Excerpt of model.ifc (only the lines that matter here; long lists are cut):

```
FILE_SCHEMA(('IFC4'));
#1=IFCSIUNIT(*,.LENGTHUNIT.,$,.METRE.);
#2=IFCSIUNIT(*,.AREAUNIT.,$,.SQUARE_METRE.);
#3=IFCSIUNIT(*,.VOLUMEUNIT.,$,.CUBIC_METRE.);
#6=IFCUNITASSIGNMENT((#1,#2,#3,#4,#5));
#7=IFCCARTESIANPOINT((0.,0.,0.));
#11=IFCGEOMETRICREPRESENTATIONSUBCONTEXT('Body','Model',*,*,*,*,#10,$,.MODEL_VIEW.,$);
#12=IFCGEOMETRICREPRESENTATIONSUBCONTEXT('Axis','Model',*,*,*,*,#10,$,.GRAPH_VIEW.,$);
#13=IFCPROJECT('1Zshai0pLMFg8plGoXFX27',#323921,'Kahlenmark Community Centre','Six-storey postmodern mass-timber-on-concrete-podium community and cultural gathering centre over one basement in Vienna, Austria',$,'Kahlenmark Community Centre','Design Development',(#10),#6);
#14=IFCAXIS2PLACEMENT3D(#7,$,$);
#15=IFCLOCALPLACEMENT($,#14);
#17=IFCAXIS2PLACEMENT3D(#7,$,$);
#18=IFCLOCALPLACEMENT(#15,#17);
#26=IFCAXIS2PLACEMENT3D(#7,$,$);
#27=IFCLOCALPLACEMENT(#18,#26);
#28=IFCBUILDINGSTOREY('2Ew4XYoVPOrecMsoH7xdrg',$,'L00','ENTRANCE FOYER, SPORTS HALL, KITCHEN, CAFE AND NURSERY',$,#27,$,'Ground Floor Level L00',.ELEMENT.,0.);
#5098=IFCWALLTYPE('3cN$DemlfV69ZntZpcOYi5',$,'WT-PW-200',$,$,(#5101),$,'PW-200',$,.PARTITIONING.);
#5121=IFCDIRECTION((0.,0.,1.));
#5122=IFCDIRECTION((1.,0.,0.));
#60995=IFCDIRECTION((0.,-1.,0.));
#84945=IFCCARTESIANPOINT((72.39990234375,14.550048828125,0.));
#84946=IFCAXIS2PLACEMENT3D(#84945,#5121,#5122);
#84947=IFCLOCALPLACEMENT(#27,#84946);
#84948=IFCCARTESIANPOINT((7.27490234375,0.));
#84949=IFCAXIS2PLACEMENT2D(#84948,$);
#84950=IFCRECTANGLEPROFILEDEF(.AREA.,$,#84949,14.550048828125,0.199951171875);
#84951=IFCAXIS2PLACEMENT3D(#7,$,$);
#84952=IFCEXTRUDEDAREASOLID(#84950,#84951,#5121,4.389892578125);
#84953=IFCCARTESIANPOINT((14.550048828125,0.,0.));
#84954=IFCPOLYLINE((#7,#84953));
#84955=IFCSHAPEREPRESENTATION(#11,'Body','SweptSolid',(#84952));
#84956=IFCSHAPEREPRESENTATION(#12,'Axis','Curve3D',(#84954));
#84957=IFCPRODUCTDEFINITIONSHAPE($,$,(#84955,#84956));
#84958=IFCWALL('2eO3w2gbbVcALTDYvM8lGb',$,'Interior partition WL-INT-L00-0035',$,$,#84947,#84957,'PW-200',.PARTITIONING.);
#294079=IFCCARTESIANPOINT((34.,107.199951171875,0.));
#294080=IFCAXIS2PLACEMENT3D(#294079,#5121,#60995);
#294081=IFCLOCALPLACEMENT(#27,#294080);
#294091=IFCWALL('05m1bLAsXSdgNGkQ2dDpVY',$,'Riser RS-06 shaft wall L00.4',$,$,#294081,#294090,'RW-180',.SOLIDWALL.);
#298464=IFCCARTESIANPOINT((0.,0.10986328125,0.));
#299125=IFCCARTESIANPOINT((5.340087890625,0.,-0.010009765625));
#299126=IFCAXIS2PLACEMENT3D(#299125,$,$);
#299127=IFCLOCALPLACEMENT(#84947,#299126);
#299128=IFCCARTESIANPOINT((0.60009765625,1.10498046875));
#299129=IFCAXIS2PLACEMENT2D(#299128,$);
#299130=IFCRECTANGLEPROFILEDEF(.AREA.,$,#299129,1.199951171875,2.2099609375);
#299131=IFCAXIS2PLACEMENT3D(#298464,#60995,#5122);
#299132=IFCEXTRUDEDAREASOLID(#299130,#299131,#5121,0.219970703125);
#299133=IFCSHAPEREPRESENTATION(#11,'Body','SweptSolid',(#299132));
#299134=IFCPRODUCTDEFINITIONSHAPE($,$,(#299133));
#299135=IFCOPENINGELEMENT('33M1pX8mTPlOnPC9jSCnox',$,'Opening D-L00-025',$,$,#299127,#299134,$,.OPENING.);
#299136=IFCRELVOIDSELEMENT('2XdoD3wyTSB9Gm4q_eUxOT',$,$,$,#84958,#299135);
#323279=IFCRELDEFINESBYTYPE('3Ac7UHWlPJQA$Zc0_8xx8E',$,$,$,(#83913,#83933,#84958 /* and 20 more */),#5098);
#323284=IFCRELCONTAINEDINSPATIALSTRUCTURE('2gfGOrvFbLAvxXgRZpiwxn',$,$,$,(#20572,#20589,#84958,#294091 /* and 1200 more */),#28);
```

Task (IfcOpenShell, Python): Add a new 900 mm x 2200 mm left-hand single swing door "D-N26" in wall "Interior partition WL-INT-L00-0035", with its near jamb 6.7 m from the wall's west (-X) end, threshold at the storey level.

```python
import numpy as np
import ifcopenshell
import ifcopenshell.api.feature
import ifcopenshell.api.geometry
import ifcopenshell.api.root
import ifcopenshell.api.spatial
import ifcopenshell.geom
import ifcopenshell.util.element
import ifcopenshell.util.placement
import ifcopenshell.util.representation
import ifcopenshell.util.shape
import ifcopenshell.util.unit

model = ifcopenshell.open("model.ifc")
unit_scale = ifcopenshell.util.unit.calculate_unit_scale(model)
settings = ifcopenshell.geom.settings()


def volume(element):
    """Net volume in cubic metres, openings subtracted."""
    shape = ifcopenshell.geom.create_shape(settings, element)
    return ifcopenshell.util.shape.get_volume(shape.geometry)


wall = model.by_guid("2eO3w2gbbVcALTDYvM8lGb")
storey = ifcopenshell.util.element.get_container(wall, ifc_class="IfcBuildingStorey")
context = ifcopenshell.util.representation.get_context(model, "Model", "Body", "MODEL_VIEW")
before = volume(wall)

width, height, from_end, sill = 0.9, 2.2, 6.7, 0.0  # metres

# The wall runs along its own X axis, and the end named is its -X end.
wall_shape = ifcopenshell.geom.create_shape(settings, wall)
x, y, z = ifcopenshell.util.shape.get_vertices(wall_shape.geometry).T
start = x.min() + from_end
face, thickness = float(y.min()), float(y.max() - y.min())
wall_matrix = ifcopenshell.util.placement.get_local_placement(wall.ObjectPlacement)
level = ifcopenshell.util.placement.get_local_placement(storey.ObjectPlacement)[2, 3]


def in_wall(x, y):
    """Placement at x, y metres in the wall's axes, at sill height."""
    matrix = wall_matrix.copy()
    matrix[:, 3] = wall_matrix @ np.array([x / unit_scale, y / unit_scale, 0.0, 1.0])
    matrix[2, 3] = level + sill / unit_scale
    return matrix


# Opening: a box that overshoots both wall faces by 50 mm.
opening = ifcopenshell.api.root.create_entity(model, ifc_class="IfcOpeningElement", predefined_type="OPENING")
box = ifcopenshell.api.geometry.add_wall_representation(
    model, context=context, length=width, height=height, thickness=thickness + 0.1
)
ifcopenshell.api.geometry.assign_representation(model, product=opening, representation=box)
ifcopenshell.api.geometry.edit_object_placement(model, product=opening, matrix=in_wall(start, face - 0.05), is_si=False)
ifcopenshell.api.feature.add_feature(model, feature=opening, element=wall)

door = ifcopenshell.api.root.create_entity(model, ifc_class="IfcDoor", name="D-N26", predefined_type="DOOR")
door.OverallWidth, door.OverallHeight = width / unit_scale, height / unit_scale
door.OperationType = "SINGLE_SWING_LEFT"
body = ifcopenshell.api.geometry.add_door_representation(
    model,
    context=context,
    overall_width=door.OverallWidth,
    overall_height=door.OverallHeight,
    operation_type="SINGLE_SWING_LEFT",
    lining_properties={"LiningDepth": thickness / unit_scale, "ThresholdDepth": thickness / unit_scale},
)
ifcopenshell.api.geometry.assign_representation(model, product=door, representation=body)
ifcopenshell.api.spatial.assign_container(model, products=[door], relating_structure=storey)
ifcopenshell.api.feature.add_filling(model, opening=opening, element=door)

# The lining spans the wall, so the door starts at the wall face.
ifcopenshell.api.geometry.edit_object_placement(model, product=door, matrix=in_wall(start, face), is_si=False)

after = volume(wall)

print(f"wall volume {before:.3f} -> {after:.3f} m3")

model.write("model_rev.ifc")
```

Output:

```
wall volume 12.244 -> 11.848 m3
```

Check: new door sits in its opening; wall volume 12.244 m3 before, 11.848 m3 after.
